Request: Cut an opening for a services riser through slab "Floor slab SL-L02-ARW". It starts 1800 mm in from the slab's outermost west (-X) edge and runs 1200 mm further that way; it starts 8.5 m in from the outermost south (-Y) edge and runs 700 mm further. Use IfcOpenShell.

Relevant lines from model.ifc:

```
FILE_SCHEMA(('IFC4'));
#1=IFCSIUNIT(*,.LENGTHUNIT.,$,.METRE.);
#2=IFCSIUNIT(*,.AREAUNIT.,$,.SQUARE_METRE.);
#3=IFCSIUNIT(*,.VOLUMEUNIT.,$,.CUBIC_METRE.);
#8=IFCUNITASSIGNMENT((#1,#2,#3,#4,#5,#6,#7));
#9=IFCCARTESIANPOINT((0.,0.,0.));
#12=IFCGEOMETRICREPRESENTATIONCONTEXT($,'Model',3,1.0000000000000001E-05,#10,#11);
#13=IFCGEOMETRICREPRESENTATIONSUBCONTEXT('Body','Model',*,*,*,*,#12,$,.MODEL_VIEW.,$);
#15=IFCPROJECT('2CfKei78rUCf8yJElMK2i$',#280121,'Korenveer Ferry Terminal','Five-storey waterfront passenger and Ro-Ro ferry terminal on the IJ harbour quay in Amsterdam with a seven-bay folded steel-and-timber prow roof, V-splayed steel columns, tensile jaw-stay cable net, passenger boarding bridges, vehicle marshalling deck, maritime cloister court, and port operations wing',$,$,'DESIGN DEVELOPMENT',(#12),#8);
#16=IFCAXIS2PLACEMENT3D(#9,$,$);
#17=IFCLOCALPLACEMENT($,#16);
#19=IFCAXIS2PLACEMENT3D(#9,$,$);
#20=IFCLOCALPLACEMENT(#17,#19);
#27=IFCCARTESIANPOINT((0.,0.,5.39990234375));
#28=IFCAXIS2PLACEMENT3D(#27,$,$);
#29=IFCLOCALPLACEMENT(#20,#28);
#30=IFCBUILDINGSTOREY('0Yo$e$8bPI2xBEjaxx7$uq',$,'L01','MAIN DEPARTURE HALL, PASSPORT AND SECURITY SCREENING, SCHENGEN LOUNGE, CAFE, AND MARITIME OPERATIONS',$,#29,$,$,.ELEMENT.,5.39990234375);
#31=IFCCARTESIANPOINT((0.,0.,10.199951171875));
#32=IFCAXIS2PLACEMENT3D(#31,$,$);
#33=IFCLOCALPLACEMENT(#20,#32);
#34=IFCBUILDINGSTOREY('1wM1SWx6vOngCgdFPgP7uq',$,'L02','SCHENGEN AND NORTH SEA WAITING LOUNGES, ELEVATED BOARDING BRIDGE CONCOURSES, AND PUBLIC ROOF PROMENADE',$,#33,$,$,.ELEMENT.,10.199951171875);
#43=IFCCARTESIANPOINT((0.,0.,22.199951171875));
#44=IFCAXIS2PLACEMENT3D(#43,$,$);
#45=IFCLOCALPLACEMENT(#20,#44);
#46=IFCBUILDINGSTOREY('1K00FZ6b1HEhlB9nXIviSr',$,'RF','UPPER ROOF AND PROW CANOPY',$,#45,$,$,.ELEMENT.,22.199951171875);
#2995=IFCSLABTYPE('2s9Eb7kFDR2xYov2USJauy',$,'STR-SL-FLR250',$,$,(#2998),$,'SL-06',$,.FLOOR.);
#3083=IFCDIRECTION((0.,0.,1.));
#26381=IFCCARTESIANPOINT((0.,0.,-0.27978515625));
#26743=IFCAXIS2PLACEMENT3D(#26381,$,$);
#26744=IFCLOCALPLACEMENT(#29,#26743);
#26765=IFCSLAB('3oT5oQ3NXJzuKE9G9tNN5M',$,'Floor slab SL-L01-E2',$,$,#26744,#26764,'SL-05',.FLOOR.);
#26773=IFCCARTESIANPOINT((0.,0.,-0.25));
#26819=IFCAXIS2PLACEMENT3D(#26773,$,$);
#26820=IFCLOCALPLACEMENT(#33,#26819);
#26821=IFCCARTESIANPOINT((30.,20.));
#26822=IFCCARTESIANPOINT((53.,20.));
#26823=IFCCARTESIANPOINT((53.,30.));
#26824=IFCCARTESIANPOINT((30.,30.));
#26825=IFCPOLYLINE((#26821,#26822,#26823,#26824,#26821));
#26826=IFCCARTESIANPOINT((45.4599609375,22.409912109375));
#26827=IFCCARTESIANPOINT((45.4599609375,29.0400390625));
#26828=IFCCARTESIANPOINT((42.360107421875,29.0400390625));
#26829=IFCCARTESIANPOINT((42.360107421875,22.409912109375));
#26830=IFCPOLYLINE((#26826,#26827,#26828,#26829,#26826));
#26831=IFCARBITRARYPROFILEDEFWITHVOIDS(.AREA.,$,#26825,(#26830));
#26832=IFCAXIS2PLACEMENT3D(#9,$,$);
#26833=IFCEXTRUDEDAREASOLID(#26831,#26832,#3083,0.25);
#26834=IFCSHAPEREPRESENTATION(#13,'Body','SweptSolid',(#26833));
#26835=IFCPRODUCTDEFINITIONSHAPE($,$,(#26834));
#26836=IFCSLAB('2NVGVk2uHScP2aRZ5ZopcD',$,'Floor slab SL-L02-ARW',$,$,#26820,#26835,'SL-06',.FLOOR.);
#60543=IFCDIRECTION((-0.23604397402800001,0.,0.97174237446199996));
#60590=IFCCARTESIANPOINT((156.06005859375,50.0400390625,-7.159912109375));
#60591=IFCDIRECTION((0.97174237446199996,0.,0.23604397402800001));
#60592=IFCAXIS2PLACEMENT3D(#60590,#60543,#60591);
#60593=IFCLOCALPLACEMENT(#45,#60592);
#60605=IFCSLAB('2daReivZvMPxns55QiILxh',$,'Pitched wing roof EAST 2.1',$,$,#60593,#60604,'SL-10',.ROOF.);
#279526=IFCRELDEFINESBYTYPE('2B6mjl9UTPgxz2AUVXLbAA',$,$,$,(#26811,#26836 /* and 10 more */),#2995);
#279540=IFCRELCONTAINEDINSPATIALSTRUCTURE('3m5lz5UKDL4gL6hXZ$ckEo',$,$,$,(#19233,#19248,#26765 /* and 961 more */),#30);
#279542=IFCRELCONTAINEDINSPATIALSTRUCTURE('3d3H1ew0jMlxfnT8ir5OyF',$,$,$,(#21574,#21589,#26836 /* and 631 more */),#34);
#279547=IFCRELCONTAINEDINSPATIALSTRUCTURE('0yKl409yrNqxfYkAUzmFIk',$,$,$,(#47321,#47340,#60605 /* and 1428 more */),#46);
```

```python
import numpy as np
import ifcopenshell
import ifcopenshell.api.feature
import ifcopenshell.api.geometry
import ifcopenshell.api.root
import ifcopenshell.geom
import ifcopenshell.util.placement
import ifcopenshell.util.representation
import ifcopenshell.util.shape
import ifcopenshell.util.unit

model = ifcopenshell.open("model.ifc")
unit_scale = ifcopenshell.util.unit.calculate_unit_scale(model)
settings = ifcopenshell.geom.settings()


def volume(element):
    """Net volume in cubic metres, openings subtracted."""
    shape = ifcopenshell.geom.create_shape(settings, element)
    return ifcopenshell.util.shape.get_volume(shape.geometry)


slab = model.by_guid("2NVGVk2uHScP2aRZ5ZopcD")
before = volume(slab)

# Extent in the slab's own axes, in metres. The edges named are its -X and -Y sides.
slab_shape = ifcopenshell.geom.create_shape(settings, slab)
vertices = ifcopenshell.util.shape.get_vertices(slab_shape.geometry)
x_min, y_min, bottom = vertices.min(axis=0)
top = vertices[:, 2].max()

opening = ifcopenshell.api.root.create_entity(model, ifc_class="IfcOpeningElement", name="Services riser opening", predefined_type="OPENING")
context = ifcopenshell.util.representation.get_context(model, "Model", "Body", "MODEL_VIEW")
width, depth = 1.2, 0.7
outline = [(0.0, 0.0), (width, 0.0), (width, depth), (0.0, depth), (0.0, 0.0)]
# Overshoot both faces by 50 mm so the cut is clean.
shape = ifcopenshell.api.geometry.add_slab_representation(
    model, context=context, depth=top - bottom + 0.1, polyline=outline
)
ifcopenshell.api.geometry.assign_representation(model, product=opening, representation=shape)

matrix = ifcopenshell.util.placement.get_local_placement(slab.ObjectPlacement)
matrix[:, 3] = matrix @ np.append(np.array([x_min + 1.8, y_min + 8.5, bottom - 0.05]) / unit_scale, 1.0)
ifcopenshell.api.geometry.edit_object_placement(model, product=opening, matrix=matrix, is_si=False)
ifcopenshell.api.feature.add_feature(model, feature=opening, element=slab)

after = volume(slab)

print(f"slab volume {before:.3f} -> {after:.3f} m3")

model.write("model_v2.ifc")
```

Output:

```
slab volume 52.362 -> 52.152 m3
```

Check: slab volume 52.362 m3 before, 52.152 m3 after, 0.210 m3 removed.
